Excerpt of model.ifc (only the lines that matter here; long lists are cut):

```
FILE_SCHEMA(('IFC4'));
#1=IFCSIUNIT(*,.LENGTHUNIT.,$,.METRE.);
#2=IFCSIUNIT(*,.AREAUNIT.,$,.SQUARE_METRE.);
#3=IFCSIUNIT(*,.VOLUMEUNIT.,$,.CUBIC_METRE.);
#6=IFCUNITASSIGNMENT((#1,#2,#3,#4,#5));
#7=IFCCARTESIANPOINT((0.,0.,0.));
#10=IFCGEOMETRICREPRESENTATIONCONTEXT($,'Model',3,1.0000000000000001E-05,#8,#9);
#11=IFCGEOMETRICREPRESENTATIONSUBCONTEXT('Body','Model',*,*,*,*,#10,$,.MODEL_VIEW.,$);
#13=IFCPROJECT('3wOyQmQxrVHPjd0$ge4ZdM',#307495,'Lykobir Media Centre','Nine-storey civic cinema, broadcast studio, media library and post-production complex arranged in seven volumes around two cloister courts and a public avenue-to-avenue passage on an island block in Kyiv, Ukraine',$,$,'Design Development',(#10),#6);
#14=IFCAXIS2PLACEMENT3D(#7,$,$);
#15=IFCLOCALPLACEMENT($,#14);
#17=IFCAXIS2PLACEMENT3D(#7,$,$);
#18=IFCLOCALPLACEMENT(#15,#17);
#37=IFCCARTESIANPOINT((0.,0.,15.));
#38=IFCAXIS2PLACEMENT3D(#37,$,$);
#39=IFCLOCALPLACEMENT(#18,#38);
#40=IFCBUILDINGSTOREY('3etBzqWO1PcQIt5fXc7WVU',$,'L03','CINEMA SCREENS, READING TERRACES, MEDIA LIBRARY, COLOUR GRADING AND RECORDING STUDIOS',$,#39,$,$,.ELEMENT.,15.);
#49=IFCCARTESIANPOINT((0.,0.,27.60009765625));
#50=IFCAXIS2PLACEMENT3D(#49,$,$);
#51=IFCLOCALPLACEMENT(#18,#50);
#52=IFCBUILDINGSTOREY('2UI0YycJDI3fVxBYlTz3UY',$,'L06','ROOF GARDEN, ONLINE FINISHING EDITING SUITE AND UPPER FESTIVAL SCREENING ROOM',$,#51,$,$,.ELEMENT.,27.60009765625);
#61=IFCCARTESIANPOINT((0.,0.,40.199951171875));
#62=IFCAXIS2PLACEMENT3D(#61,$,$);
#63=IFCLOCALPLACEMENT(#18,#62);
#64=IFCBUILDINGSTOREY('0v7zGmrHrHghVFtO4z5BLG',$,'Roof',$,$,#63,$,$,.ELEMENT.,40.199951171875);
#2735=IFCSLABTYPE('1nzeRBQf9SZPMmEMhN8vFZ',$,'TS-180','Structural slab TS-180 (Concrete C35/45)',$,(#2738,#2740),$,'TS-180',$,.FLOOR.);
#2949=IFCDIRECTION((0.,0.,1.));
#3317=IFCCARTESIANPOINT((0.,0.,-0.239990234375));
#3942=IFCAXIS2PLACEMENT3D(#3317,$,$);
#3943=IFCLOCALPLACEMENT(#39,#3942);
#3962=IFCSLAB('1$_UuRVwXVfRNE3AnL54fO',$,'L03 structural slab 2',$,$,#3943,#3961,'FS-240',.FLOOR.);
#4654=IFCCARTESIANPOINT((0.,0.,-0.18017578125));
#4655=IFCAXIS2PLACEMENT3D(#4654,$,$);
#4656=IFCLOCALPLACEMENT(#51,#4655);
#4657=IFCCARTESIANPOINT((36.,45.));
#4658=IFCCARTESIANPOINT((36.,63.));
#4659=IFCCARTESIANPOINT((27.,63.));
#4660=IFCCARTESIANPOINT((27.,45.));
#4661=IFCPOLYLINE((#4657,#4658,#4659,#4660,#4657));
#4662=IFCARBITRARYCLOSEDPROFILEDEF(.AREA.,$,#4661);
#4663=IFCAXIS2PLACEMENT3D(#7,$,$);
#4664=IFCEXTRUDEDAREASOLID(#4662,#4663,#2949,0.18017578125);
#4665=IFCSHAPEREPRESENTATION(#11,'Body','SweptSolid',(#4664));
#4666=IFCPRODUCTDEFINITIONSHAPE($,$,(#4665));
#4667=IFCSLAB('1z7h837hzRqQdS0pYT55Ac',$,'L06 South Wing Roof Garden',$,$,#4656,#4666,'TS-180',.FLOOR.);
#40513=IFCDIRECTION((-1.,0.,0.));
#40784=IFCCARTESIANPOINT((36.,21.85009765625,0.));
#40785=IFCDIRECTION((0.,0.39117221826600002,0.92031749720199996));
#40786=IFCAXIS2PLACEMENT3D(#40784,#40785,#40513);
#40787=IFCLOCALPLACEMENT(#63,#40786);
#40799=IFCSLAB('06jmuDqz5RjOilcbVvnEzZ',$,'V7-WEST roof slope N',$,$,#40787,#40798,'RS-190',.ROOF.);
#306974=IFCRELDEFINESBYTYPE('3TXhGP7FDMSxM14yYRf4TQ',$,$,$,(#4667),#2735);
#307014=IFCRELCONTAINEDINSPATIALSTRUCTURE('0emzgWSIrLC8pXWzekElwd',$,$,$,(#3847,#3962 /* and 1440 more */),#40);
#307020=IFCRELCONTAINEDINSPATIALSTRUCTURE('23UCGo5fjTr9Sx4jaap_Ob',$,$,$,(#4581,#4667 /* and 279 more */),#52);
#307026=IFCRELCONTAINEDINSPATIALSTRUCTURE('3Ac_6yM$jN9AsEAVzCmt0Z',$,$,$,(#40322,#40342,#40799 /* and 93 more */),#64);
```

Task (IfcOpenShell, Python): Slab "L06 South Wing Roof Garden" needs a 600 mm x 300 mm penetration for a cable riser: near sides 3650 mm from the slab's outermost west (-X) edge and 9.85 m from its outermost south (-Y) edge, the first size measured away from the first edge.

```python
import numpy as np
import ifcopenshell
import ifcopenshell.api.feature
import ifcopenshell.api.geometry
import ifcopenshell.api.root
import ifcopenshell.geom
import ifcopenshell.util.placement
import ifcopenshell.util.representation
import ifcopenshell.util.shape
import ifcopenshell.util.unit

model = ifcopenshell.open("model.ifc")
unit_scale = ifcopenshell.util.unit.calculate_unit_scale(model)
settings = ifcopenshell.geom.settings()


def volume(element):
    """Net volume in cubic metres, openings subtracted."""
    shape = ifcopenshell.geom.create_shape(settings, element)
    return ifcopenshell.util.shape.get_volume(shape.geometry)


slab = model.by_guid("1z7h837hzRqQdS0pYT55Ac")
before = volume(slab)

# Extent in the slab's own axes, in metres. The edges named are its -X and -Y sides.
slab_shape = ifcopenshell.geom.create_shape(settings, slab)
vertices = ifcopenshell.util.shape.get_vertices(slab_shape.geometry)
x_min, y_min, bottom = vertices.min(axis=0)
top = vertices[:, 2].max()

opening = ifcopenshell.api.root.create_entity(model, ifc_class="IfcOpeningElement", name="Cable riser opening", predefined_type="OPENING")
context = ifcopenshell.util.representation.get_context(model, "Model", "Body", "MODEL_VIEW")
width, depth = 0.6, 0.3
outline = [(0.0, 0.0), (width, 0.0), (width, depth), (0.0, depth), (0.0, 0.0)]
# Overshoot both faces by 50 mm so the cut is clean.
shape = ifcopenshell.api.geometry.add_slab_representation(
    model, context=context, depth=top - bottom + 0.1, polyline=outline
)
ifcopenshell.api.geometry.assign_representation(model, product=opening, representation=shape)

matrix = ifcopenshell.util.placement.get_local_placement(slab.ObjectPlacement)
matrix[:, 3] = matrix @ np.append(np.array([x_min + 3.65, y_min + 9.85, bottom - 0.05]) / unit_scale, 1.0)
ifcopenshell.api.geometry.edit_object_placement(model, product=opening, matrix=matrix, is_si=False)
ifcopenshell.api.feature.add_feature(model, feature=opening, element=slab)

after = volume(slab)

print(f"slab volume {before:.3f} -> {after:.3f} m3")

model.write("model-out.ifc")
```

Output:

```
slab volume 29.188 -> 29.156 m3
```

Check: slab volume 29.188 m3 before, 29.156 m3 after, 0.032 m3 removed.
